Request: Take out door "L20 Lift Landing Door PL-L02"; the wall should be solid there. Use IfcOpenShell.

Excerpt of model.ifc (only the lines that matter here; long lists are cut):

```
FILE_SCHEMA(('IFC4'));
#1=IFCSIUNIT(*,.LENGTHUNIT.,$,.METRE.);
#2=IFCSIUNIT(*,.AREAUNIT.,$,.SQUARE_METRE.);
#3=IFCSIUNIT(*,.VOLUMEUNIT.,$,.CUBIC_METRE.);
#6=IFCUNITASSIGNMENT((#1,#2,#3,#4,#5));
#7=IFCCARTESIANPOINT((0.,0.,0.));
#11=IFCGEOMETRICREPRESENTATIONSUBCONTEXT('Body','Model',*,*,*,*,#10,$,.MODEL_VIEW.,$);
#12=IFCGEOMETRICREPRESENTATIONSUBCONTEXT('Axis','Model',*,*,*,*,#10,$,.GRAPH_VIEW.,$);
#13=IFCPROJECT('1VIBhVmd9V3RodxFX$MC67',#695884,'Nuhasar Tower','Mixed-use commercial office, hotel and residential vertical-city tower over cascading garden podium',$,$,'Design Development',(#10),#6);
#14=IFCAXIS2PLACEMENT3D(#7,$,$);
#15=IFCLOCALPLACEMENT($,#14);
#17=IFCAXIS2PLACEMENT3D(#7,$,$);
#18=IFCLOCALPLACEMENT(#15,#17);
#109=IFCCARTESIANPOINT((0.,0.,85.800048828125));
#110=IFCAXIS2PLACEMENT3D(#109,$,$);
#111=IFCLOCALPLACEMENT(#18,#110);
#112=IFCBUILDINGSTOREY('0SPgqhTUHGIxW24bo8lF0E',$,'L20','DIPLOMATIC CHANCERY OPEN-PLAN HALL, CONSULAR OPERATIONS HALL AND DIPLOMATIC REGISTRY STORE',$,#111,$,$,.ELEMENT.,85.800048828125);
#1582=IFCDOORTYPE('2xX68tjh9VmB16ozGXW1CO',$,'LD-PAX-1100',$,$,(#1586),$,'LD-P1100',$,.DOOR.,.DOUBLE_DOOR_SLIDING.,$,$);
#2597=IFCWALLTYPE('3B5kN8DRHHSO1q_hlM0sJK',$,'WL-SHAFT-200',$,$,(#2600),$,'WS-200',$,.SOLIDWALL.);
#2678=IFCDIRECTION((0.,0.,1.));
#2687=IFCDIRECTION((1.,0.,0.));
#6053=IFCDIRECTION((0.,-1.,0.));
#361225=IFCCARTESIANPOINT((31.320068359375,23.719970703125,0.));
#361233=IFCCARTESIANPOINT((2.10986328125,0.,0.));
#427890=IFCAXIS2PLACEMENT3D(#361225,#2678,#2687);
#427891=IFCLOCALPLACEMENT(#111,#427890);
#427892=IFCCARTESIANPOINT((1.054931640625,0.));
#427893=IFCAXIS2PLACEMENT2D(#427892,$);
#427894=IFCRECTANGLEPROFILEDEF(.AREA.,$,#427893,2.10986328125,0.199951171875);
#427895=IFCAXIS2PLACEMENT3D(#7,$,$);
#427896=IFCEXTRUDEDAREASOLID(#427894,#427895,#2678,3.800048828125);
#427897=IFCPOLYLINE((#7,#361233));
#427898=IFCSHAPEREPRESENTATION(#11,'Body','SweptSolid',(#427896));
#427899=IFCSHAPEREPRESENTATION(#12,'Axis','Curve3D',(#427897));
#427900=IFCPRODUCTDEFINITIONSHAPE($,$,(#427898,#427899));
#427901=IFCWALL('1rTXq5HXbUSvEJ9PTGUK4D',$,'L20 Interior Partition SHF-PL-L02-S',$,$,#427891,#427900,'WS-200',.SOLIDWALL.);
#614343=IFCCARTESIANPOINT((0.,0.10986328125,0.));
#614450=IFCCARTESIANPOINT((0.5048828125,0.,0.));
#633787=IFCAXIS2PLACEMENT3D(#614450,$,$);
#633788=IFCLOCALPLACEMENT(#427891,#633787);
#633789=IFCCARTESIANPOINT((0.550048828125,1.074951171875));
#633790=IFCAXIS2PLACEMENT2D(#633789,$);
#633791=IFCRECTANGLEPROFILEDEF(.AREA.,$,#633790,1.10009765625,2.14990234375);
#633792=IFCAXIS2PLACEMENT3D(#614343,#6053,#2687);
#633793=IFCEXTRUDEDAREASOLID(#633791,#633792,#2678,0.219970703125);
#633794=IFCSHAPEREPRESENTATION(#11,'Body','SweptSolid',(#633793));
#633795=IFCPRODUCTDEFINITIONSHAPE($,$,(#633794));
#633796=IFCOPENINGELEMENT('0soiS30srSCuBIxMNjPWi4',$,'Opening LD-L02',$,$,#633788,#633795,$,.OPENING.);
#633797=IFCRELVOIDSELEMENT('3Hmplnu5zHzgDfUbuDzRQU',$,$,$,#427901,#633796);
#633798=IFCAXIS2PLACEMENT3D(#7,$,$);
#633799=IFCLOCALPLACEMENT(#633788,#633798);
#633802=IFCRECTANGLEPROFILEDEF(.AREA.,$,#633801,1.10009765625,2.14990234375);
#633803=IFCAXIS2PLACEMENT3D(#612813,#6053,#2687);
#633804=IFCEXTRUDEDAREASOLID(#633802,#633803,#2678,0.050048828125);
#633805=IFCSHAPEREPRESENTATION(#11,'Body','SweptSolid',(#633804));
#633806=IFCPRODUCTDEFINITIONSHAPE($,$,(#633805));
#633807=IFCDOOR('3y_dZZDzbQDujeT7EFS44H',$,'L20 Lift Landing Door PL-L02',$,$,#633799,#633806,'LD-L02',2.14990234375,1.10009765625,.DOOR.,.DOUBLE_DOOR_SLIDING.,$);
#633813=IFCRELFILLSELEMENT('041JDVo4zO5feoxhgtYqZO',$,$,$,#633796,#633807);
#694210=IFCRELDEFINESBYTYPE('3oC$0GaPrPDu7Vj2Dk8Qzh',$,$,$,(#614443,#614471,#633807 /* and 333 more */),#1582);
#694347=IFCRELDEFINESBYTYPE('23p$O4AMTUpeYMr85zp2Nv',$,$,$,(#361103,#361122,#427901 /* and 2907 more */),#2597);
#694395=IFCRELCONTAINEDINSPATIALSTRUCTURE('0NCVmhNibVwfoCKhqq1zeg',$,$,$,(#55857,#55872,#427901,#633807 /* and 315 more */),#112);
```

```python
import ifcopenshell
import ifcopenshell.api.feature
import ifcopenshell.api.root
import ifcopenshell.geom
import ifcopenshell.util.shape

model = ifcopenshell.open("model.ifc")
settings = ifcopenshell.geom.settings()


def volume(element):
    """Net volume in cubic metres, openings subtracted."""
    shape = ifcopenshell.geom.create_shape(settings, element)
    return ifcopenshell.util.shape.get_volume(shape.geometry)


door = model.by_guid("3y_dZZDzbQDujeT7EFS44H")
opening = door.FillsVoids[0].RelatingOpeningElement
wall = opening.VoidsElements[0].RelatingBuildingElement
before = volume(wall)

ifcopenshell.api.root.remove_product(model, product=door)
ifcopenshell.api.feature.remove_feature(model, feature=opening)

after = volume(wall)

print(f"wall volume {before:.3f} -> {after:.3f} m3")

model.write("model_edited.ifc")
```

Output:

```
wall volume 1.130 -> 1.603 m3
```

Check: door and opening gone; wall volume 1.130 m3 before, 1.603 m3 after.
